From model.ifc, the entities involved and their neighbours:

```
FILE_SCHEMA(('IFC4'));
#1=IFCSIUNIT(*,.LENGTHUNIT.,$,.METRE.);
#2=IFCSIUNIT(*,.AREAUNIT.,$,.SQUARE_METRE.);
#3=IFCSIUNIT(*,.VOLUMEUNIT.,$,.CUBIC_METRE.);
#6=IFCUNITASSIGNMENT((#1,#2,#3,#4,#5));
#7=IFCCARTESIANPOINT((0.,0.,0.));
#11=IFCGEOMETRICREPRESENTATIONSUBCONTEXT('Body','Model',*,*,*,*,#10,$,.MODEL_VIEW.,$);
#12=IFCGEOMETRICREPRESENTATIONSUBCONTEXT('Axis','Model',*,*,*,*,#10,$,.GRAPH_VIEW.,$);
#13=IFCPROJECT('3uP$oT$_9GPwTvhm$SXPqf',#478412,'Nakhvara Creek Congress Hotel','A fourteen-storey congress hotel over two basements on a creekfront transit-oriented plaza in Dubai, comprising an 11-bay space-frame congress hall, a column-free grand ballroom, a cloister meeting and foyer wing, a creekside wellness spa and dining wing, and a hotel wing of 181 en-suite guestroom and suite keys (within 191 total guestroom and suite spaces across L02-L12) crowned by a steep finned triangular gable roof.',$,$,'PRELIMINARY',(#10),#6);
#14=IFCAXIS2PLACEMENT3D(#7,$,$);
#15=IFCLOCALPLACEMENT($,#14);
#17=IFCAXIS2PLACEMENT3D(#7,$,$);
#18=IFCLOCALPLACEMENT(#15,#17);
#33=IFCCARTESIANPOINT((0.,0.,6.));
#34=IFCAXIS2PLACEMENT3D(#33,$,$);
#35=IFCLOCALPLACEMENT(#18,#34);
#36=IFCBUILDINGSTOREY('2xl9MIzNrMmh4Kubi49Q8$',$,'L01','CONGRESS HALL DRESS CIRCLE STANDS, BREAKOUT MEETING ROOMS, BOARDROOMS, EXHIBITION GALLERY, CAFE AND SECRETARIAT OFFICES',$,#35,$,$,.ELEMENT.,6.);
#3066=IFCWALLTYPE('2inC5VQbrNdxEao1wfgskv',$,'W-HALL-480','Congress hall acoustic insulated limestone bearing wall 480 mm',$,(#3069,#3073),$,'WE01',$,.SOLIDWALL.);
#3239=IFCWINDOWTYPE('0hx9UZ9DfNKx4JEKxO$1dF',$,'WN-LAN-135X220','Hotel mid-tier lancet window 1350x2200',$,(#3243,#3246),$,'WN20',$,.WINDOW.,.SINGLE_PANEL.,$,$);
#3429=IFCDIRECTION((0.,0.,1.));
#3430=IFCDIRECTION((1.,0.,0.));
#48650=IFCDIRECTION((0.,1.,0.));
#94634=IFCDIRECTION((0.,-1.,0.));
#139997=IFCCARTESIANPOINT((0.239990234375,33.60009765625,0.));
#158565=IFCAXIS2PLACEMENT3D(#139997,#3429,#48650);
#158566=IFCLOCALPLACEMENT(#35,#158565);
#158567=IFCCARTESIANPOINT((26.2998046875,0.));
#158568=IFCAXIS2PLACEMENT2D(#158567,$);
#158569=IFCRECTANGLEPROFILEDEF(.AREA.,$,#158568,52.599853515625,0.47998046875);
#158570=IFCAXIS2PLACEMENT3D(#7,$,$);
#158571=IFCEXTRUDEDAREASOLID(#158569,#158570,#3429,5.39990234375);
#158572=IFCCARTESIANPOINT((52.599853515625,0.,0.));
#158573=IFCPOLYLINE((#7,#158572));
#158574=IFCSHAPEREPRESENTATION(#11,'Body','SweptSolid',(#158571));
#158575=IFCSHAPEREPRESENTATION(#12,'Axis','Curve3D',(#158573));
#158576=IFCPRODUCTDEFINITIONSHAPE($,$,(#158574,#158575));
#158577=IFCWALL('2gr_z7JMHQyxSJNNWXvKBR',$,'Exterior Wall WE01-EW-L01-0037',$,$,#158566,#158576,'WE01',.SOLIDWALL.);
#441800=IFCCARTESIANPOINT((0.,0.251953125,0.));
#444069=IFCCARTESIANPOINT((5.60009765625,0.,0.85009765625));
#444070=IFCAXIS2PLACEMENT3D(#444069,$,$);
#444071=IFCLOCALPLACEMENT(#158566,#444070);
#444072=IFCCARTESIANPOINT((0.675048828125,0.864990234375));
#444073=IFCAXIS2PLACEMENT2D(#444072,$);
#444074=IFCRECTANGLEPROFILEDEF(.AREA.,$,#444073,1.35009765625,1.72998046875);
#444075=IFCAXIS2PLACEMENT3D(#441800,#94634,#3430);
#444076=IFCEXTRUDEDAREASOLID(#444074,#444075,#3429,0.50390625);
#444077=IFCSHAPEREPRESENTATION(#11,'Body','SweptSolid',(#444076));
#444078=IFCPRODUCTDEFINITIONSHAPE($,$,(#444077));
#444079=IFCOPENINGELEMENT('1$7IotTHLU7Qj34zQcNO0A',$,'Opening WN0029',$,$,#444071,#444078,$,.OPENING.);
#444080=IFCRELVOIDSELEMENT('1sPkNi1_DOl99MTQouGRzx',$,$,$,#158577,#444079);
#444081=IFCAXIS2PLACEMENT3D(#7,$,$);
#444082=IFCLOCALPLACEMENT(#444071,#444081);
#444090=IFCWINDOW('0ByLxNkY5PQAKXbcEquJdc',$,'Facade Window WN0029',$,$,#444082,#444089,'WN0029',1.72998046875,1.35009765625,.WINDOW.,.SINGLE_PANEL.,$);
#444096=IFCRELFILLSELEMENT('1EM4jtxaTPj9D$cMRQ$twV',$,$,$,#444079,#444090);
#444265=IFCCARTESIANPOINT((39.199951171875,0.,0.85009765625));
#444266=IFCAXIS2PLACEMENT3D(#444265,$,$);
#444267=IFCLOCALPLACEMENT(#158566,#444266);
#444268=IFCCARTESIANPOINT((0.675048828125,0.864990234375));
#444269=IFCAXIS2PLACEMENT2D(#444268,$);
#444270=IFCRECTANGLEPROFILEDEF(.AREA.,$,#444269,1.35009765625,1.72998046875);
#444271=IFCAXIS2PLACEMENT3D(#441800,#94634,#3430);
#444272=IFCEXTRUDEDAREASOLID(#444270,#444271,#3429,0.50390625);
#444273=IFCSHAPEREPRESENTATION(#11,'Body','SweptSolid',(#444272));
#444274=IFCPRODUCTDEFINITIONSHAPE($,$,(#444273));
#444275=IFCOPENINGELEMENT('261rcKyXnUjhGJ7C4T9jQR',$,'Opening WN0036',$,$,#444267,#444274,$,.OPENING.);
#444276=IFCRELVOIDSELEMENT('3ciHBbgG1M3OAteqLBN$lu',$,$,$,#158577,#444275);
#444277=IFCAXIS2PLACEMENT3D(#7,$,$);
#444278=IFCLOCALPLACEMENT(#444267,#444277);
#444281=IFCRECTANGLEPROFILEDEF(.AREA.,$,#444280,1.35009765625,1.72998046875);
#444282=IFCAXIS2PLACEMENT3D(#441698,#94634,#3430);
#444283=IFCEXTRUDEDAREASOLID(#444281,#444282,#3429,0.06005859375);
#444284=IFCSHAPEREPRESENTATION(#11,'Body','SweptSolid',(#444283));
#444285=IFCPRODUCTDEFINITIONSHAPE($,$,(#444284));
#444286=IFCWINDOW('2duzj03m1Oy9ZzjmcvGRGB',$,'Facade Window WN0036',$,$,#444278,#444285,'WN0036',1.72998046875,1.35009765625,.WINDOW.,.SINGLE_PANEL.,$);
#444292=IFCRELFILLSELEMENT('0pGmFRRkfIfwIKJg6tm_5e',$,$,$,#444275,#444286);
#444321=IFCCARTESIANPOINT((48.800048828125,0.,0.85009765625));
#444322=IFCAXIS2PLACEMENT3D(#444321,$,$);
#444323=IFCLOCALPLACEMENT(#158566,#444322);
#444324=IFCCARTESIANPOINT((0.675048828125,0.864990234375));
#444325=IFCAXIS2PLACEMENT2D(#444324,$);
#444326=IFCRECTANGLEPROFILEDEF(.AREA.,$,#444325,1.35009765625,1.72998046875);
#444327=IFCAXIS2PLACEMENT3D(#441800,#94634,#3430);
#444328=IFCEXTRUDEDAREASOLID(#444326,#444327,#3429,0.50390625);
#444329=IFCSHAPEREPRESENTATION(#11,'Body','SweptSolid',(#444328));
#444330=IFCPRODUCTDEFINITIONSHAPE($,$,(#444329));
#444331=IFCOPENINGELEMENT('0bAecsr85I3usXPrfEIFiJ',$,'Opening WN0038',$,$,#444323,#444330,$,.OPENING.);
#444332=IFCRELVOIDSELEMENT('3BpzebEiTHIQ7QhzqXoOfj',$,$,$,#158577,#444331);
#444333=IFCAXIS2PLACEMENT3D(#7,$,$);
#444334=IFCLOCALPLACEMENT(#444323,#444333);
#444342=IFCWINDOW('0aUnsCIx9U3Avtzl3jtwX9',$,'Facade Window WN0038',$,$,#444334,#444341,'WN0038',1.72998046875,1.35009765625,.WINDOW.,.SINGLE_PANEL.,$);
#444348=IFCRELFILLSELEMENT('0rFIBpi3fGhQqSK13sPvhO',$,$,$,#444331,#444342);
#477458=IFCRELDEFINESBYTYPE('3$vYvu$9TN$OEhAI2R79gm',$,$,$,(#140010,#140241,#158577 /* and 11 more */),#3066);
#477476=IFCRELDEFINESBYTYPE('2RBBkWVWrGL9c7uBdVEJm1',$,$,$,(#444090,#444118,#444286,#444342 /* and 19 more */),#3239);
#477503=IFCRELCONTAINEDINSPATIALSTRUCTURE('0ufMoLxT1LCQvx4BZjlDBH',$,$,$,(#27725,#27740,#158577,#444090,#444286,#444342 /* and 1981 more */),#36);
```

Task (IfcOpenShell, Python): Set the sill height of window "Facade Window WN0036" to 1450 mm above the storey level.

```python
import numpy as np
import ifcopenshell
import ifcopenshell.api.geometry
import ifcopenshell.geom
import ifcopenshell.util.element
import ifcopenshell.util.placement
import ifcopenshell.util.shape
import ifcopenshell.util.unit

model = ifcopenshell.open("model.ifc")
unit_scale = ifcopenshell.util.unit.calculate_unit_scale(model)

window = model.by_guid("2duzj03m1Oy9ZzjmcvGRGB")
opening = window.FillsVoids[0].RelatingOpeningElement
storey = ifcopenshell.util.element.get_container(window, ifc_class="IfcBuildingStorey")
level = ifcopenshell.util.placement.get_local_placement(storey.ObjectPlacement)[2, 3]

# The opening's origin need not be at the sill, so measure its lowest point.
shape = ifcopenshell.geom.create_shape(ifcopenshell.geom.settings(), opening)
bottom = ifcopenshell.util.shape.get_shape_bottom_elevation(shape, shape.geometry) / unit_scale
dz = level + 1.45 / unit_scale - bottom

shift = np.array([0.0, 0.0, dz])
# The window is placed relative to its opening, so it follows when the opening moves.
matrix = ifcopenshell.util.placement.get_local_placement(opening.ObjectPlacement)
matrix[:3, 3] += shift
ifcopenshell.api.geometry.edit_object_placement(
    model, product=opening, matrix=matrix, is_si=False, should_transform_children=True
)

print(f"moved by {dz * unit_scale:+.3f} m")

model.write("model_v2.ifc")
```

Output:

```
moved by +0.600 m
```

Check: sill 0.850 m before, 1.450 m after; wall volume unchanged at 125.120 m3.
